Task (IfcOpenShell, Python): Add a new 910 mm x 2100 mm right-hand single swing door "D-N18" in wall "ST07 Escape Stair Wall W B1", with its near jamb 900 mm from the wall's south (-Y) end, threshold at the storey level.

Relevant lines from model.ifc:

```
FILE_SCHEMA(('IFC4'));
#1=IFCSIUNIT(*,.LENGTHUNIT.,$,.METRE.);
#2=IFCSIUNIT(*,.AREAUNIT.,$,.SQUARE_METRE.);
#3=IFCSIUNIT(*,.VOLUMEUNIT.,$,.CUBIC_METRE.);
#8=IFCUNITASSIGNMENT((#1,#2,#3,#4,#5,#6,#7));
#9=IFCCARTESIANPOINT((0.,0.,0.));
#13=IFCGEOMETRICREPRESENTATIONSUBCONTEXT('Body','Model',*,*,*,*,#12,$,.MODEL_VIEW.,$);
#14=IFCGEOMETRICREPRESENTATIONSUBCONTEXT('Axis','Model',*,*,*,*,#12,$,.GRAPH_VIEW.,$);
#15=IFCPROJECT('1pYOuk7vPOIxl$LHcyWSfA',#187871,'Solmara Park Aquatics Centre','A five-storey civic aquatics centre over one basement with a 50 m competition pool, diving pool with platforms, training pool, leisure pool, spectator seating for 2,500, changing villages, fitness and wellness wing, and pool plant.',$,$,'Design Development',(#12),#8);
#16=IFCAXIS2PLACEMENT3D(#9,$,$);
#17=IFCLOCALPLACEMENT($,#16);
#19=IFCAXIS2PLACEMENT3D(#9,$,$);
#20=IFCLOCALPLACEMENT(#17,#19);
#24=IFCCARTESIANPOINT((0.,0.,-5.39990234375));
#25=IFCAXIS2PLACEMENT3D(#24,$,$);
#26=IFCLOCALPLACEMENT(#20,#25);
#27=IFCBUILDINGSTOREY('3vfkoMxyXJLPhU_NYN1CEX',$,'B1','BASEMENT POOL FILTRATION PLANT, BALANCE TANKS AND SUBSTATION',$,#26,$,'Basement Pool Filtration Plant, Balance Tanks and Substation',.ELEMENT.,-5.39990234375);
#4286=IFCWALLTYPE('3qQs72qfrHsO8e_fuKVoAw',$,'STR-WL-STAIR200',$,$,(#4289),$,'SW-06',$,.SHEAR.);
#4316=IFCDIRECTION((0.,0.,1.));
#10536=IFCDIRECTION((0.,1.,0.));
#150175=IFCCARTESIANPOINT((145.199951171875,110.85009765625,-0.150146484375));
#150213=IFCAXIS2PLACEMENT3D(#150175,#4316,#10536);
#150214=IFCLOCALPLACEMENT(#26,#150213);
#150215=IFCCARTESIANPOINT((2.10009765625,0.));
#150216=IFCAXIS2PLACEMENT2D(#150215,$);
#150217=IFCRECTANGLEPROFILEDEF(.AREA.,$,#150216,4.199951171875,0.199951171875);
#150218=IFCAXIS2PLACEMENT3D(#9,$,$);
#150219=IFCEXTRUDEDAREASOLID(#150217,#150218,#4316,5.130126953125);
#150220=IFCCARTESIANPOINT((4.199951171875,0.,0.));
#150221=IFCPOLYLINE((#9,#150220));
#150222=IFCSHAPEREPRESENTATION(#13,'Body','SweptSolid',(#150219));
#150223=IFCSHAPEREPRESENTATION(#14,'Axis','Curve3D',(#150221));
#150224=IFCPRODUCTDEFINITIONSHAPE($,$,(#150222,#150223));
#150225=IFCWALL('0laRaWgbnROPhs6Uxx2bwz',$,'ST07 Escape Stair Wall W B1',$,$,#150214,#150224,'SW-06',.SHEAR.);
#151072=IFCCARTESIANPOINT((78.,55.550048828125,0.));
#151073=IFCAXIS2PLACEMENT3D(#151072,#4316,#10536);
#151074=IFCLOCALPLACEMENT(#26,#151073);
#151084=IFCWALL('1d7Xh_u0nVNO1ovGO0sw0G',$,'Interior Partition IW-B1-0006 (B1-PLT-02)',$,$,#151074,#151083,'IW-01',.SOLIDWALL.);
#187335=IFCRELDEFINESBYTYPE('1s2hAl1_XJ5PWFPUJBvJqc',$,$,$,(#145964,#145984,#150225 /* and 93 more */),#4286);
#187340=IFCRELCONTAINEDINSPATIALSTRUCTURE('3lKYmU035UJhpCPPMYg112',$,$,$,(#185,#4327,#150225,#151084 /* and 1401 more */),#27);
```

```python
import numpy as np
import ifcopenshell
import ifcopenshell.api.feature
import ifcopenshell.api.geometry
import ifcopenshell.api.root
import ifcopenshell.api.spatial
import ifcopenshell.geom
import ifcopenshell.util.element
import ifcopenshell.util.placement
import ifcopenshell.util.representation
import ifcopenshell.util.shape
import ifcopenshell.util.unit

model = ifcopenshell.open("model.ifc")
unit_scale = ifcopenshell.util.unit.calculate_unit_scale(model)
settings = ifcopenshell.geom.settings()


def volume(element):
    """Net volume in cubic metres, openings subtracted."""
    shape = ifcopenshell.geom.create_shape(settings, element)
    return ifcopenshell.util.shape.get_volume(shape.geometry)


wall = model.by_guid("0laRaWgbnROPhs6Uxx2bwz")
storey = ifcopenshell.util.element.get_container(wall, ifc_class="IfcBuildingStorey")
context = ifcopenshell.util.representation.get_context(model, "Model", "Body", "MODEL_VIEW")
before = volume(wall)

width, height, from_end, sill = 0.91, 2.1, 0.9, 0.0  # metres

# The wall runs along its own X axis, and the end named is its -X end.
wall_shape = ifcopenshell.geom.create_shape(settings, wall)
x, y, z = ifcopenshell.util.shape.get_vertices(wall_shape.geometry).T
start = x.min() + from_end
face, thickness = float(y.min()), float(y.max() - y.min())
wall_matrix = ifcopenshell.util.placement.get_local_placement(wall.ObjectPlacement)
level = ifcopenshell.util.placement.get_local_placement(storey.ObjectPlacement)[2, 3]


def in_wall(x, y):
    """Placement at x, y metres in the wall's axes, at sill height."""
    matrix = wall_matrix.copy()
    matrix[:, 3] = wall_matrix @ np.array([x / unit_scale, y / unit_scale, 0.0, 1.0])
    matrix[2, 3] = level + sill / unit_scale
    return matrix


# Opening: a box that overshoots both wall faces by 50 mm.
opening = ifcopenshell.api.root.create_entity(model, ifc_class="IfcOpeningElement", predefined_type="OPENING")
box = ifcopenshell.api.geometry.add_wall_representation(
    model, context=context, length=width, height=height, thickness=thickness + 0.1
)
ifcopenshell.api.geometry.assign_representation(model, product=opening, representation=box)
ifcopenshell.api.geometry.edit_object_placement(model, product=opening, matrix=in_wall(start, face - 0.05), is_si=False)
ifcopenshell.api.feature.add_feature(model, feature=opening, element=wall)

door = ifcopenshell.api.root.create_entity(model, ifc_class="IfcDoor", name="D-N18", predefined_type="DOOR")
door.OverallWidth, door.OverallHeight = width / unit_scale, height / unit_scale
door.OperationType = "SINGLE_SWING_RIGHT"
body = ifcopenshell.api.geometry.add_door_representation(
    model,
    context=context,
    overall_width=door.OverallWidth,
    overall_height=door.OverallHeight,
    operation_type="SINGLE_SWING_RIGHT",
    lining_properties={"LiningDepth": thickness / unit_scale, "ThresholdDepth": thickness / unit_scale},
)
ifcopenshell.api.geometry.assign_representation(model, product=door, representation=body)
ifcopenshell.api.spatial.assign_container(model, products=[door], relating_structure=storey)
ifcopenshell.api.feature.add_filling(model, opening=opening, element=door)

# The lining spans the wall, so the door starts at the wall face.
ifcopenshell.api.geometry.edit_object_placement(model, product=door, matrix=in_wall(start, face), is_si=False)

after = volume(wall)

print(f"wall volume {before:.3f} -> {after:.3f} m3")

model.write("model-out.ifc")
```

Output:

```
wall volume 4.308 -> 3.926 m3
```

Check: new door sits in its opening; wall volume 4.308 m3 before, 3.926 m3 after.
